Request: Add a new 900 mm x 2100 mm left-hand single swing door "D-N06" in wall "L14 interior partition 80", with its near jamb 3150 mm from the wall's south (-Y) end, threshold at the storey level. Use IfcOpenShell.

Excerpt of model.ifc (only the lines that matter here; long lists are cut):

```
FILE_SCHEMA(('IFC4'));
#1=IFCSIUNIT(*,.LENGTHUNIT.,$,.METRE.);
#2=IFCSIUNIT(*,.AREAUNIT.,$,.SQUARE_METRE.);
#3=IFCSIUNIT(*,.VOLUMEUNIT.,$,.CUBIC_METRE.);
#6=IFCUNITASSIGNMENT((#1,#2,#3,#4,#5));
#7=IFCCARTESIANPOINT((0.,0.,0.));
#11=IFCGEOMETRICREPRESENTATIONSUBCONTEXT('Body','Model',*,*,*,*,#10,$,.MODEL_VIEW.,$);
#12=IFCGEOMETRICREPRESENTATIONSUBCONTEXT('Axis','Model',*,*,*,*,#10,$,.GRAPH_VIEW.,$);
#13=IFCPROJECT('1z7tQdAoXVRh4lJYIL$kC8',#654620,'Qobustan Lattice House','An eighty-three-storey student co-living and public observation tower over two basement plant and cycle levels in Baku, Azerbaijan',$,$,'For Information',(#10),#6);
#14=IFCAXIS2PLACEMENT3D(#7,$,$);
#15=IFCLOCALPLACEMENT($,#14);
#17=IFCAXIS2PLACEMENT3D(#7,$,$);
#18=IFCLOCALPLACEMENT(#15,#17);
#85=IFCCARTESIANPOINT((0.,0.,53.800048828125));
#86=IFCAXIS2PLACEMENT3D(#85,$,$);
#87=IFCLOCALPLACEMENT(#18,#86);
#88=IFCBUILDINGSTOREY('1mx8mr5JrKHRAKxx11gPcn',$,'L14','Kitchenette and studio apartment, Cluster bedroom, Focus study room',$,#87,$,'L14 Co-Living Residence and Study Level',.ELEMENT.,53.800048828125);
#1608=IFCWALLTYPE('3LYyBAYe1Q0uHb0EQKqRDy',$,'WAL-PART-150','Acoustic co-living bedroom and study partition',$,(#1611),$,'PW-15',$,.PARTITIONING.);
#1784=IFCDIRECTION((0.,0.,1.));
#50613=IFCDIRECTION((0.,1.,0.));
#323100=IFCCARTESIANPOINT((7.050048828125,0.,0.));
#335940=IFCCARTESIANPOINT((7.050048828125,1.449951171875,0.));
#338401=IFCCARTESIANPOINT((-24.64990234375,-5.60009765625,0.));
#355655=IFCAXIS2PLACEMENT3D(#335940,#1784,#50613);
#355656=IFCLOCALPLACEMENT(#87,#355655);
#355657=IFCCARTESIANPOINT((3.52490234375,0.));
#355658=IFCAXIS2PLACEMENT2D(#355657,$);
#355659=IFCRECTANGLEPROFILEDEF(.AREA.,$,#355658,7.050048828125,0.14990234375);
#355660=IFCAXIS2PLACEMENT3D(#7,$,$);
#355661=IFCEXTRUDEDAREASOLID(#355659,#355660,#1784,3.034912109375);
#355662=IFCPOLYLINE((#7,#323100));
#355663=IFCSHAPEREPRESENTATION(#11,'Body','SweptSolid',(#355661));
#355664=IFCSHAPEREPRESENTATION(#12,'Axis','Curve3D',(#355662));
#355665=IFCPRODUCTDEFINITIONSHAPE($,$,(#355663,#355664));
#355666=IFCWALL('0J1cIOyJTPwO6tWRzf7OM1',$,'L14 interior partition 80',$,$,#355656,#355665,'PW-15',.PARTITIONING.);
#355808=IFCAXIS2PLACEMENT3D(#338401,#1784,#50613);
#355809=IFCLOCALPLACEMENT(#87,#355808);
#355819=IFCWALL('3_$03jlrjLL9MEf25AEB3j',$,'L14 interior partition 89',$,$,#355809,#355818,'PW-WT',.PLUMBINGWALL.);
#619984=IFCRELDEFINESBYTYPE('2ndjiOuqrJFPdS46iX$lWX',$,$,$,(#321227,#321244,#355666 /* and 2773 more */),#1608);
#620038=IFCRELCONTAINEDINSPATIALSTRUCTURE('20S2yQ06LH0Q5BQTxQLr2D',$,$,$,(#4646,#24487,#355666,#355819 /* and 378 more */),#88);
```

```python
import numpy as np
import ifcopenshell
import ifcopenshell.api.feature
import ifcopenshell.api.geometry
import ifcopenshell.api.root
import ifcopenshell.api.spatial
import ifcopenshell.geom
import ifcopenshell.util.element
import ifcopenshell.util.placement
import ifcopenshell.util.representation
import ifcopenshell.util.shape
import ifcopenshell.util.unit

model = ifcopenshell.open("model.ifc")
unit_scale = ifcopenshell.util.unit.calculate_unit_scale(model)
settings = ifcopenshell.geom.settings()


def volume(element):
    """Net volume in cubic metres, openings subtracted."""
    shape = ifcopenshell.geom.create_shape(settings, element)
    return ifcopenshell.util.shape.get_volume(shape.geometry)


wall = model.by_id(355666)
storey = ifcopenshell.util.element.get_container(wall, ifc_class="IfcBuildingStorey")
context = ifcopenshell.util.representation.get_context(model, "Model", "Body", "MODEL_VIEW")
before = volume(wall)

width, height, from_end, sill = 0.9, 2.1, 3.15, 0.0  # metres

# The wall runs along its own X axis, and the end named is its -X end.
wall_shape = ifcopenshell.geom.create_shape(settings, wall)
x, y, z = ifcopenshell.util.shape.get_vertices(wall_shape.geometry).T
start = x.min() + from_end
face, thickness = float(y.min()), float(y.max() - y.min())
wall_matrix = ifcopenshell.util.placement.get_local_placement(wall.ObjectPlacement)
level = ifcopenshell.util.placement.get_local_placement(storey.ObjectPlacement)[2, 3]


def in_wall(x, y):
    """Placement at x, y metres in the wall's axes, at sill height."""
    matrix = wall_matrix.copy()
    matrix[:, 3] = wall_matrix @ np.array([x / unit_scale, y / unit_scale, 0.0, 1.0])
    matrix[2, 3] = level + sill / unit_scale
    return matrix


# Opening: a box that overshoots both wall faces by 50 mm.
opening = ifcopenshell.api.root.create_entity(model, ifc_class="IfcOpeningElement", predefined_type="OPENING")
box = ifcopenshell.api.geometry.add_wall_representation(
    model, context=context, length=width, height=height, thickness=thickness + 0.1
)
ifcopenshell.api.geometry.assign_representation(model, product=opening, representation=box)
ifcopenshell.api.geometry.edit_object_placement(model, product=opening, matrix=in_wall(start, face - 0.05), is_si=False)
ifcopenshell.api.feature.add_feature(model, feature=opening, element=wall)

door = ifcopenshell.api.root.create_entity(model, ifc_class="IfcDoor", name="D-N06", predefined_type="DOOR")
door.OverallWidth, door.OverallHeight = width / unit_scale, height / unit_scale
door.OperationType = "SINGLE_SWING_LEFT"
body = ifcopenshell.api.geometry.add_door_representation(
    model,
    context=context,
    overall_width=door.OverallWidth,
    overall_height=door.OverallHeight,
    operation_type="SINGLE_SWING_LEFT",
    lining_properties={"LiningDepth": thickness / unit_scale, "ThresholdDepth": thickness / unit_scale},
)
ifcopenshell.api.geometry.assign_representation(model, product=door, representation=body)
ifcopenshell.api.spatial.assign_container(model, products=[door], relating_structure=storey)
ifcopenshell.api.feature.add_filling(model, opening=opening, element=door)

# The lining spans the wall, so the door starts at the wall face.
ifcopenshell.api.geometry.edit_object_placement(model, product=door, matrix=in_wall(start, face), is_si=False)

after = volume(wall)

print(f"wall volume {before:.3f} -> {after:.3f} m3")

model.write("model_rev.ifc")
```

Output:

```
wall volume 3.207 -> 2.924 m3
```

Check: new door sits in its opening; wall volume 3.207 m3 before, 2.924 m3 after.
